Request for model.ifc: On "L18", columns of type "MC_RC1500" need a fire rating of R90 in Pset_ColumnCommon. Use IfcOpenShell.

First a look at what the model holds.

```python
import ifcopenshell
import ifcopenshell.util.element

model = ifcopenshell.open("model.ifc")
print(model.schema)
storey = next(s for s in model.by_type("IfcBuildingStorey") if s.Name == "L18")
columns = [e for e in ifcopenshell.util.element.get_decomposition(storey) if e.is_a("IfcColumn")]
seen = {}
for e in columns:
    element_type = ifcopenshell.util.element.get_type(e)
    key = (element_type.Name if element_type != e and element_type else None, ifcopenshell.util.element.get_pset(e, "Pset_ColumnCommon", "FireRating"))
    seen[key] = seen.get(key, 0) + 1
for (name, value), count in sorted(seen.items(), key=str):
    print(count, "x", name, "|", value)
```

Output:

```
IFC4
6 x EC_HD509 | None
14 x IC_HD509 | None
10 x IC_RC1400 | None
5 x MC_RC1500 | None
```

```python
import ifcopenshell
import ifcopenshell.api.pset
import ifcopenshell.util.element

model = ifcopenshell.open("model.ifc")

storey = next(s for s in model.by_type("IfcBuildingStorey") if s.Name == "L18")
columns = [e for e in ifcopenshell.util.element.get_decomposition(storey) if e.is_a("IfcColumn")]

count = 0
for e in columns:
    element_type = ifcopenshell.util.element.get_type(e)
    if element_type in (None, e) or element_type.Name != "MC_RC1500":
        continue
    # add_pset returns the element's existing set when there is one.
    pset = ifcopenshell.api.pset.add_pset(model, product=e, name="Pset_ColumnCommon")
    ifcopenshell.api.pset.edit_pset(model, pset=pset, properties={"FireRating": "R90"})
    count += 1

print(count, "columns updated")

model.write("model_updated.ifc")
```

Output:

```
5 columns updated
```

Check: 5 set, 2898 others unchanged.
